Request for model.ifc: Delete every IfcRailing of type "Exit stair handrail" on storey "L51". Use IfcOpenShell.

First a look at what the model holds.

```python
import ifcopenshell
import ifcopenshell.util.element

model = ifcopenshell.open("model.ifc")
print(model.schema)
storey = next(s for s in model.by_type("IfcBuildingStorey") if s.Name == "L51")
railings = [e for e in ifcopenshell.util.element.get_decomposition(storey) if e.is_a("IfcRailing")]
seen = {}
for e in railings:
    element_type = ifcopenshell.util.element.get_type(e)
    name = element_type.Name if element_type not in (None, e) else None
    seen[name] = seen.get(name, 0) + 1
for name, count in sorted(seen.items(), key=str):
    print(count, "x", name)
```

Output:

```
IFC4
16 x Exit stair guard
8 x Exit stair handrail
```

```python
import ifcopenshell
import ifcopenshell.api.root
import ifcopenshell.util.element

model = ifcopenshell.open("model.ifc")

storey = next(s for s in model.by_type("IfcBuildingStorey") if s.Name == "L51")
railings = [e for e in ifcopenshell.util.element.get_decomposition(storey) if e.is_a("IfcRailing")]
targets = [e for e in railings if (t := ifcopenshell.util.element.get_type(e)) not in (None, e) and t.Name == "Exit stair handrail"]

for e in targets:
    ifcopenshell.api.root.remove_product(model, product=e)
print(len(targets), "removed")

model.write("model_v2.ifc")
```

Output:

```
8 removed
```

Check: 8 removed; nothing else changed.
